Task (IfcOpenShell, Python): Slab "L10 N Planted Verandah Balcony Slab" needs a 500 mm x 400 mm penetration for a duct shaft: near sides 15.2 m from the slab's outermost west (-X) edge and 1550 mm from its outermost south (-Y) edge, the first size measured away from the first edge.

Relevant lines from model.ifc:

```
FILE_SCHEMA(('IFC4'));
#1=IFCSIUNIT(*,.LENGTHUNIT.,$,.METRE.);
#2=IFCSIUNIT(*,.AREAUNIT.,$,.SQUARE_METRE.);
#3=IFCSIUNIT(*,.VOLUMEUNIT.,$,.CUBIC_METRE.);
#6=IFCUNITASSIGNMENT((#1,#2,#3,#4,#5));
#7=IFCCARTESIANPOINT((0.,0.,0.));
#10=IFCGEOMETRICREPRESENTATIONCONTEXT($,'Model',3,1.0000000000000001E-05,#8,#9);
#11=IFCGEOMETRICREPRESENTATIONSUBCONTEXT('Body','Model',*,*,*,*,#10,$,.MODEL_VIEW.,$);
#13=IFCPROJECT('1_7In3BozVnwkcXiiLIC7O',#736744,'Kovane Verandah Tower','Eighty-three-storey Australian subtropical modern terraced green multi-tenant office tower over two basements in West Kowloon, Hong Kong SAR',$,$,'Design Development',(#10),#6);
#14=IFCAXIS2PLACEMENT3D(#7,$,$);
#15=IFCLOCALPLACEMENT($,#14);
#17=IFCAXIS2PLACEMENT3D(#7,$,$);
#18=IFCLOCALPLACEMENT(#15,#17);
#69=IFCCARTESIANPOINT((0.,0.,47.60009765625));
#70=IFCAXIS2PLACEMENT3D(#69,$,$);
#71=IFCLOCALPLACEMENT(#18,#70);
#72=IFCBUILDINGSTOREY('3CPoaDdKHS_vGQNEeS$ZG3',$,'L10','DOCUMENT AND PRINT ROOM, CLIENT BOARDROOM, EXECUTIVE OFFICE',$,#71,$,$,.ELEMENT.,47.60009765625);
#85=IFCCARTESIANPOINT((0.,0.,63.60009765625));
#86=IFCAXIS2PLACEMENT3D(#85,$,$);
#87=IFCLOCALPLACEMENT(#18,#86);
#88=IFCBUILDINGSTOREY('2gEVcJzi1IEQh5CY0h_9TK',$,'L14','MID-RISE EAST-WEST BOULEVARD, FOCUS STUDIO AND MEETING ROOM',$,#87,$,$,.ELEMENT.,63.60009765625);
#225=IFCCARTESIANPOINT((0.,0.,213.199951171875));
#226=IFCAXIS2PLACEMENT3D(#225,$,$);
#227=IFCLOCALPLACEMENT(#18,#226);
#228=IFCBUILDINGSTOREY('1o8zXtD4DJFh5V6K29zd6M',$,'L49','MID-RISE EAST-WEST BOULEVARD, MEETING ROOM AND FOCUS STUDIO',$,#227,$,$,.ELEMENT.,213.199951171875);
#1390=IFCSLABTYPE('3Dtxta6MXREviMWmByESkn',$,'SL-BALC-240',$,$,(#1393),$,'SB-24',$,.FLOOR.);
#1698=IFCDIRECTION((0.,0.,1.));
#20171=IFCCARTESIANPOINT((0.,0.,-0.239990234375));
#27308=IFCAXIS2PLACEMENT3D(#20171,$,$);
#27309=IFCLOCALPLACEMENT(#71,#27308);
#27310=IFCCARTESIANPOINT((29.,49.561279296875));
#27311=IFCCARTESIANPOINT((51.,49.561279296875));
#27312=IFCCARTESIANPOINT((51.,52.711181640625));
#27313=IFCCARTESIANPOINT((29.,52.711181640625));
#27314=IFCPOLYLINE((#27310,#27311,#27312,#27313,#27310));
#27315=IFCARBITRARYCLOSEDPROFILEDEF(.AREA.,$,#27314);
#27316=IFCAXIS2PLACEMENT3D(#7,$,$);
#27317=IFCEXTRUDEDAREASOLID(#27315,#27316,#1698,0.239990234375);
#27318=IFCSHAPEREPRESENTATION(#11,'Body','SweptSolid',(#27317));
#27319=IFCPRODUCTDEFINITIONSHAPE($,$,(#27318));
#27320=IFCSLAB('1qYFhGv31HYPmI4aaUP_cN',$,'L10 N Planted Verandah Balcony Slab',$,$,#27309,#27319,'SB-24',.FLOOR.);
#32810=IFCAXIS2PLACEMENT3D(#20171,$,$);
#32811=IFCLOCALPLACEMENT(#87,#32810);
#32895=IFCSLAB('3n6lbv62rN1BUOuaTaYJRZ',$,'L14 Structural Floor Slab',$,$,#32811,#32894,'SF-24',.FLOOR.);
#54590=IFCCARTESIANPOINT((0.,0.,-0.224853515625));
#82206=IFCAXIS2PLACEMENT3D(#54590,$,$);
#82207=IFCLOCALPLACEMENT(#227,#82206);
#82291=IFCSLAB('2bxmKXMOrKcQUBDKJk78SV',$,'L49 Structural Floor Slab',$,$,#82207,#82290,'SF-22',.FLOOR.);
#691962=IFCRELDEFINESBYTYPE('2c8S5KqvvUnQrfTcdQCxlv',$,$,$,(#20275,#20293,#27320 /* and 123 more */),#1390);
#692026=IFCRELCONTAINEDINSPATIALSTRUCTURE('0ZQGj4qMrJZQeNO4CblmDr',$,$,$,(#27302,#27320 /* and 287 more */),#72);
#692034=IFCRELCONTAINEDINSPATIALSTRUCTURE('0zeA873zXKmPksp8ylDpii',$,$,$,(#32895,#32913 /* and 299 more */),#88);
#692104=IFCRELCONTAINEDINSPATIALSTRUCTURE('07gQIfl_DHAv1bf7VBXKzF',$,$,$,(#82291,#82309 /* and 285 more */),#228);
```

```python
import numpy as np
import ifcopenshell
import ifcopenshell.api.feature
import ifcopenshell.api.geometry
import ifcopenshell.api.root
import ifcopenshell.geom
import ifcopenshell.util.placement
import ifcopenshell.util.representation
import ifcopenshell.util.shape
import ifcopenshell.util.unit

model = ifcopenshell.open("model.ifc")
unit_scale = ifcopenshell.util.unit.calculate_unit_scale(model)
settings = ifcopenshell.geom.settings()


def volume(element):
    """Net volume in cubic metres, openings subtracted."""
    shape = ifcopenshell.geom.create_shape(settings, element)
    return ifcopenshell.util.shape.get_volume(shape.geometry)


slab = model.by_guid("1qYFhGv31HYPmI4aaUP_cN")
before = volume(slab)

# Extent in the slab's own axes, in metres. The edges named are its -X and -Y sides.
slab_shape = ifcopenshell.geom.create_shape(settings, slab)
vertices = ifcopenshell.util.shape.get_vertices(slab_shape.geometry)
x_min, y_min, bottom = vertices.min(axis=0)
top = vertices[:, 2].max()

opening = ifcopenshell.api.root.create_entity(model, ifc_class="IfcOpeningElement", name="Duct shaft opening", predefined_type="OPENING")
context = ifcopenshell.util.representation.get_context(model, "Model", "Body", "MODEL_VIEW")
width, depth = 0.5, 0.4
outline = [(0.0, 0.0), (width, 0.0), (width, depth), (0.0, depth), (0.0, 0.0)]
# Overshoot both faces by 50 mm so the cut is clean.
shape = ifcopenshell.api.geometry.add_slab_representation(
    model, context=context, depth=top - bottom + 0.1, polyline=outline
)
ifcopenshell.api.geometry.assign_representation(model, product=opening, representation=shape)

matrix = ifcopenshell.util.placement.get_local_placement(slab.ObjectPlacement)
matrix[:, 3] = matrix @ np.append(np.array([x_min + 15.2, y_min + 1.55, bottom - 0.05]) / unit_scale, 1.0)
ifcopenshell.api.geometry.edit_object_placement(model, product=opening, matrix=matrix, is_si=False)
ifcopenshell.api.feature.add_feature(model, feature=opening, element=slab)

after = volume(slab)

print(f"slab volume {before:.3f} -> {after:.3f} m3")

model.write("model_edited.ifc")
```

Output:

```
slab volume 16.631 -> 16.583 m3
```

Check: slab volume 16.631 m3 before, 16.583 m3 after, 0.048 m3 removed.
